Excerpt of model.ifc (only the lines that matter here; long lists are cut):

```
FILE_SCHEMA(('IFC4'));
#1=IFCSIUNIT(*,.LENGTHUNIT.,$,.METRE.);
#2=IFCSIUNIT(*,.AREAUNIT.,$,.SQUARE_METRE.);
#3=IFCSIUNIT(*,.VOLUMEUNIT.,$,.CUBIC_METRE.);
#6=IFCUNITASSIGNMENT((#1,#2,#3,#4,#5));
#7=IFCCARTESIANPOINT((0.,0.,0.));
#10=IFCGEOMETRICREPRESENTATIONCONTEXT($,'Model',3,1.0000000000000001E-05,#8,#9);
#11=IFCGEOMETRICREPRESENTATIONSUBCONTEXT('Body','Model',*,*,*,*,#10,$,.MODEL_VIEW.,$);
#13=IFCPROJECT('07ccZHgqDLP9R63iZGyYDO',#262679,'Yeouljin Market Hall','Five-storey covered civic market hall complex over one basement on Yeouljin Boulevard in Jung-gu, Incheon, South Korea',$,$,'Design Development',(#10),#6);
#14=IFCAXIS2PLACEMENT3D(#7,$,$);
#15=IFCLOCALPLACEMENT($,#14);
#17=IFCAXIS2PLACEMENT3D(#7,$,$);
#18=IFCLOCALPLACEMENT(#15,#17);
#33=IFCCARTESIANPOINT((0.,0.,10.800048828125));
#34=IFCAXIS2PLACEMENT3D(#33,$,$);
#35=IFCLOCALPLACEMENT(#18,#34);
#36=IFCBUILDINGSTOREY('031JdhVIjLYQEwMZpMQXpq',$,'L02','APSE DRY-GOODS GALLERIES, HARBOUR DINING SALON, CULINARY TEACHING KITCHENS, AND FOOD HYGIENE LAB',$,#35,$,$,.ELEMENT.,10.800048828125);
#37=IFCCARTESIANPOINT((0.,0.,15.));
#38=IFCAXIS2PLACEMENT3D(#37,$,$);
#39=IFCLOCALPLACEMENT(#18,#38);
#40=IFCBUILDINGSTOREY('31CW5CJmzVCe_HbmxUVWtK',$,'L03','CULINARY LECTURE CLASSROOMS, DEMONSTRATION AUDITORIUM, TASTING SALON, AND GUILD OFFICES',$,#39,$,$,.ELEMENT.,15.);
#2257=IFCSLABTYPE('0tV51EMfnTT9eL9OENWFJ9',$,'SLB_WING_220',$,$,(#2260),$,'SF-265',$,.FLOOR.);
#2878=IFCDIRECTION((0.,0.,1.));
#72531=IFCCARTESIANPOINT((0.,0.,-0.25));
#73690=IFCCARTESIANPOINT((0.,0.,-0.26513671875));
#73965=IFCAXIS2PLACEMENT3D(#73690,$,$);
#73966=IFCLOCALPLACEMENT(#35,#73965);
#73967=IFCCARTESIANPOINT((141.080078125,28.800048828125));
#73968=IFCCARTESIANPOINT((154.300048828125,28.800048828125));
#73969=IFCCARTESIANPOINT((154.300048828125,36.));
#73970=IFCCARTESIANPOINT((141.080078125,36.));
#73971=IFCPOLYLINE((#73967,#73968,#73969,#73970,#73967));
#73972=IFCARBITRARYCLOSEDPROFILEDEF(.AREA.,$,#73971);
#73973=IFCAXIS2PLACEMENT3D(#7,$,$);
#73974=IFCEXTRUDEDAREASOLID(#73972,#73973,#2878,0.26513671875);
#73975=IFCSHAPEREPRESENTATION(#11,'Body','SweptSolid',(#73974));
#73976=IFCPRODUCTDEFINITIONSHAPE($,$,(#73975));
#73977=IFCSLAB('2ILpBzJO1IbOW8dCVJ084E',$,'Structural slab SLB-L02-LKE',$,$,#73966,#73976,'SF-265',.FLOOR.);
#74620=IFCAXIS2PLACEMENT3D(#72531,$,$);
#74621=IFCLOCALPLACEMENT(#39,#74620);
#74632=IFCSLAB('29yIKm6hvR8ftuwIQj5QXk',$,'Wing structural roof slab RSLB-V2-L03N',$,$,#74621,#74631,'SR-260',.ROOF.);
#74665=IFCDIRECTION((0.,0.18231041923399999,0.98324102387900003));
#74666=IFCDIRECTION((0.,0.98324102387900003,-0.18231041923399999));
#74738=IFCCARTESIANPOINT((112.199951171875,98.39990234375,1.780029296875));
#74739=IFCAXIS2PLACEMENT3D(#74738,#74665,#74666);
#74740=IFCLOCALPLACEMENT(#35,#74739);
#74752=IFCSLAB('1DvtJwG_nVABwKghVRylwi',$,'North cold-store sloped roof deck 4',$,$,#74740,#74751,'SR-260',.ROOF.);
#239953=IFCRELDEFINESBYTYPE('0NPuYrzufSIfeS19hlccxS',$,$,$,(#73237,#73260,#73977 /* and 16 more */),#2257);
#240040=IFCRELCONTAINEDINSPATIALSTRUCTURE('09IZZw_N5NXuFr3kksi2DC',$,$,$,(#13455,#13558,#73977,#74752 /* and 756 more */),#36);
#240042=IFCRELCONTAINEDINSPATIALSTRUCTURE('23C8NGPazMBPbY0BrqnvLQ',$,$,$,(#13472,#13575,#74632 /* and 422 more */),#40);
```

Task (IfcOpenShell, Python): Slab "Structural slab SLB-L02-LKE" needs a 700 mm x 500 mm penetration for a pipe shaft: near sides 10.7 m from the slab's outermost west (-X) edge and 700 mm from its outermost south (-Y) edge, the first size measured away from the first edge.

```python
import numpy as np
import ifcopenshell
import ifcopenshell.api.feature
import ifcopenshell.api.geometry
import ifcopenshell.api.root
import ifcopenshell.geom
import ifcopenshell.util.placement
import ifcopenshell.util.representation
import ifcopenshell.util.shape
import ifcopenshell.util.unit

model = ifcopenshell.open("model.ifc")
unit_scale = ifcopenshell.util.unit.calculate_unit_scale(model)
settings = ifcopenshell.geom.settings()


def volume(element):
    """Net volume in cubic metres, openings subtracted."""
    shape = ifcopenshell.geom.create_shape(settings, element)
    return ifcopenshell.util.shape.get_volume(shape.geometry)


slab = model.by_id(73977)
before = volume(slab)

# Extent in the slab's own axes, in metres. The edges named are its -X and -Y sides.
slab_shape = ifcopenshell.geom.create_shape(settings, slab)
vertices = ifcopenshell.util.shape.get_vertices(slab_shape.geometry)
x_min, y_min, bottom = vertices.min(axis=0)
top = vertices[:, 2].max()

opening = ifcopenshell.api.root.create_entity(model, ifc_class="IfcOpeningElement", name="Pipe shaft opening", predefined_type="OPENING")
context = ifcopenshell.util.representation.get_context(model, "Model", "Body", "MODEL_VIEW")
width, depth = 0.7, 0.5
outline = [(0.0, 0.0), (width, 0.0), (width, depth), (0.0, depth), (0.0, 0.0)]
# Overshoot both faces by 50 mm so the cut is clean.
shape = ifcopenshell.api.geometry.add_slab_representation(
    model, context=context, depth=top - bottom + 0.1, polyline=outline
)
ifcopenshell.api.geometry.assign_representation(model, product=opening, representation=shape)

matrix = ifcopenshell.util.placement.get_local_placement(slab.ObjectPlacement)
matrix[:, 3] = matrix @ np.append(np.array([x_min + 10.7, y_min + 0.7, bottom - 0.05]) / unit_scale, 1.0)
ifcopenshell.api.geometry.edit_object_placement(model, product=opening, matrix=matrix, is_si=False)
ifcopenshell.api.feature.add_feature(model, feature=opening, element=slab)

after = volume(slab)

print(f"slab volume {before:.3f} -> {after:.3f} m3")

model.write("model_updated.ifc")
```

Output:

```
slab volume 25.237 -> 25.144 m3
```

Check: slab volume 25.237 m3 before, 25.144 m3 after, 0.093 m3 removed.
